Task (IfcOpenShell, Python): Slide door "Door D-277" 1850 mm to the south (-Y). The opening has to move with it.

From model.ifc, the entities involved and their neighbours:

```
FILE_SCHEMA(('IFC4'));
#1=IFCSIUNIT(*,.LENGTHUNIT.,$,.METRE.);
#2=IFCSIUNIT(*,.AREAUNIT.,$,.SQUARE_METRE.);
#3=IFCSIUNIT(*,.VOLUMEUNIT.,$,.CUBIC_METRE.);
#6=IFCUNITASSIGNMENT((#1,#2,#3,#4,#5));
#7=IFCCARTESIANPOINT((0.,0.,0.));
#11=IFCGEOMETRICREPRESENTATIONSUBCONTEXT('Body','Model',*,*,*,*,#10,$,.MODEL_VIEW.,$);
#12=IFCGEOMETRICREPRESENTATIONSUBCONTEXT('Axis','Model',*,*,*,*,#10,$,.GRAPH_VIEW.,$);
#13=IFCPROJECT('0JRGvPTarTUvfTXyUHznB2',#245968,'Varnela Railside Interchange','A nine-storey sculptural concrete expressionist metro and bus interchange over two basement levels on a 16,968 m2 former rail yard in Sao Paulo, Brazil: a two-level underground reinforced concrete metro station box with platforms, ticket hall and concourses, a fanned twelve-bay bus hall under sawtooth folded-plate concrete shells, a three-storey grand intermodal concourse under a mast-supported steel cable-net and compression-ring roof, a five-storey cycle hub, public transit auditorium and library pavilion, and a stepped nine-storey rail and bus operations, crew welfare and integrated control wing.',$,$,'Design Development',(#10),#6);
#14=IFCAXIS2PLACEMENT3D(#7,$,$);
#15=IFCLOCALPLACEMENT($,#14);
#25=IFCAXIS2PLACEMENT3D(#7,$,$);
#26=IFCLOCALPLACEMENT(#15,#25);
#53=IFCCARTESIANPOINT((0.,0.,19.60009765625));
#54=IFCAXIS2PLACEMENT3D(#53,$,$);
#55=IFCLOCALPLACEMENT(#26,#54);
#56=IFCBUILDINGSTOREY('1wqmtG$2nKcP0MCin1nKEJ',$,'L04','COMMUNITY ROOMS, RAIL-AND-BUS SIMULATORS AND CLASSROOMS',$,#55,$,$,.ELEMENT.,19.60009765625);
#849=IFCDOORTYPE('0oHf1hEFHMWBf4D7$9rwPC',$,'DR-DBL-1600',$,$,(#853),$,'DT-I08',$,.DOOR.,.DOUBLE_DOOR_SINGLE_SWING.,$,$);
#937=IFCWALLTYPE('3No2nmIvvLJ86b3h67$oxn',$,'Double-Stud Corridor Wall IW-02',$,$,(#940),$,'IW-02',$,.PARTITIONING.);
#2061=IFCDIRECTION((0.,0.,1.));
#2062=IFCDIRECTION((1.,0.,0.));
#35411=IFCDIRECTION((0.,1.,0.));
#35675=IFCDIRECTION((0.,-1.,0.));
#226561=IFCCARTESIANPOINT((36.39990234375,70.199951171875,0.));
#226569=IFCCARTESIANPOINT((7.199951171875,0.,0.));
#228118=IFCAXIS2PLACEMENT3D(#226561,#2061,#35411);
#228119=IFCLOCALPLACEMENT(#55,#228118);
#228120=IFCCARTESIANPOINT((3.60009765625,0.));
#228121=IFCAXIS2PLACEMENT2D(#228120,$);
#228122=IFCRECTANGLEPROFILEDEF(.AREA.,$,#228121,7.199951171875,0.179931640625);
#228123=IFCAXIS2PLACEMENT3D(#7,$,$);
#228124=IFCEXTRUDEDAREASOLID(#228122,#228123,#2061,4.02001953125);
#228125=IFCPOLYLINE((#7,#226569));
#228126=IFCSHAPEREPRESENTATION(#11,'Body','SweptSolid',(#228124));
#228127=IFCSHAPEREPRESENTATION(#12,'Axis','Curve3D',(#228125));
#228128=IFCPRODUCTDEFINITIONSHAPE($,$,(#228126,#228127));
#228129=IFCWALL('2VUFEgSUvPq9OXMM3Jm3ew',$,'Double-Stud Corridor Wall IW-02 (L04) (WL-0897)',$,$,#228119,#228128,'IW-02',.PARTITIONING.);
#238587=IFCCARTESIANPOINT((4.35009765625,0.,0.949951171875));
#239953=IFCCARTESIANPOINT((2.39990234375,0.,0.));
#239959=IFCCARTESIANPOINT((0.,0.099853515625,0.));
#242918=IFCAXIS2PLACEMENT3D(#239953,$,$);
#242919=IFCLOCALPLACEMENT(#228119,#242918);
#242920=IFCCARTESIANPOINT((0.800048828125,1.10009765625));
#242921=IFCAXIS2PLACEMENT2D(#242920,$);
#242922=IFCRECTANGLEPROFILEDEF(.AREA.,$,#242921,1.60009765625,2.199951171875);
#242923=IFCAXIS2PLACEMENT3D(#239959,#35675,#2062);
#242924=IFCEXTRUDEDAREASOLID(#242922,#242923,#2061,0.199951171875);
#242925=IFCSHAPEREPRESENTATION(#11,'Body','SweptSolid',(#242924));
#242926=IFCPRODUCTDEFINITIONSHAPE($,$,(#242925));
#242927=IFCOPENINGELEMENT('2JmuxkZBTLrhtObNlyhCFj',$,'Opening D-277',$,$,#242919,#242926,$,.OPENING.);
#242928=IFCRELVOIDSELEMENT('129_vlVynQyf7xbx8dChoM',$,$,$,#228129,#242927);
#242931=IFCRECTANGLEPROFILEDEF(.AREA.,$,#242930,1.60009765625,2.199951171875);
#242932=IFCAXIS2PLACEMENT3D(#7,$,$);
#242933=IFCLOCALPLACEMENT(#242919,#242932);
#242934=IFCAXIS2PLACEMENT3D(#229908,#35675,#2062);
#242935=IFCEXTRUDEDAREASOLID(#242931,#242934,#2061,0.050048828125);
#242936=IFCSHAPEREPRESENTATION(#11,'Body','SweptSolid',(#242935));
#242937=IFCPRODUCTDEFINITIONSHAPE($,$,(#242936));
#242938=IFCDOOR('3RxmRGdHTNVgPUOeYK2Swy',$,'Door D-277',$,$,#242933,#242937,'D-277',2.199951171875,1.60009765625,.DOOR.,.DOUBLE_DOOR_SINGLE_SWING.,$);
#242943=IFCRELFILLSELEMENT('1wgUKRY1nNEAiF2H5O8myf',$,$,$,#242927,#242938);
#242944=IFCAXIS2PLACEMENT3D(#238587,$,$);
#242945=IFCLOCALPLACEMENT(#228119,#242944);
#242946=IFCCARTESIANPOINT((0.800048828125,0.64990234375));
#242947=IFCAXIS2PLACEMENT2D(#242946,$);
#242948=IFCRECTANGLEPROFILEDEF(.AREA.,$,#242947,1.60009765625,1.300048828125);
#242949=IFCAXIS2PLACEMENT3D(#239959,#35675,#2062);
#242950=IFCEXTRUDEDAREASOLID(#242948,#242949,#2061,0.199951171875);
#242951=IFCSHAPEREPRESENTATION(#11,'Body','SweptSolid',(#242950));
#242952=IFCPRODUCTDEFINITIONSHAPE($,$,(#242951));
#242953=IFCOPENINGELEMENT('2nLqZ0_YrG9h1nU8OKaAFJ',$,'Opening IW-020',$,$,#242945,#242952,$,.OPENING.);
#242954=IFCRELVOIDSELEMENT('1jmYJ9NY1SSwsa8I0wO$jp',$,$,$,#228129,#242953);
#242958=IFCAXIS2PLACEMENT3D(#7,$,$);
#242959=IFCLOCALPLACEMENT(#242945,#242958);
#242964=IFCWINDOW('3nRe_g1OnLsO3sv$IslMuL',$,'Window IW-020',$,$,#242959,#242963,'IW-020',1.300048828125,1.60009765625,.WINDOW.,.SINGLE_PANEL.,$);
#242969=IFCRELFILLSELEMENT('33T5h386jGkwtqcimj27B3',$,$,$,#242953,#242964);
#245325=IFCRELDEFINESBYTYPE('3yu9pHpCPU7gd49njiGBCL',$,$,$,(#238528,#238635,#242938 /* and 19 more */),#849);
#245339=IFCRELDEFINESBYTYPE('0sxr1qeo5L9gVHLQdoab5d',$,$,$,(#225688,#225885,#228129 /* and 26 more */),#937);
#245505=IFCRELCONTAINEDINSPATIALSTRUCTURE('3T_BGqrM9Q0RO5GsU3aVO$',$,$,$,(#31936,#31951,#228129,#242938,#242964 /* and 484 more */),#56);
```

```python
import ifcopenshell
import ifcopenshell.api.geometry
import ifcopenshell.util.placement
import ifcopenshell.util.unit

model = ifcopenshell.open("model.ifc")
unit_scale = ifcopenshell.util.unit.calculate_unit_scale(model)

door = model.by_id(242938)
opening = door.FillsVoids[0].RelatingOpeningElement
wall = opening.VoidsElements[0].RelatingBuildingElement

wall_matrix = ifcopenshell.util.placement.get_local_placement(wall.ObjectPlacement)
shift = wall_matrix[:3, 0] * -1.85 / unit_scale
before = ifcopenshell.util.placement.get_local_placement(door.ObjectPlacement)[:3, 3].copy()

# The door is placed relative to its opening, so it follows when the opening moves.
matrix = ifcopenshell.util.placement.get_local_placement(opening.ObjectPlacement)
matrix[:3, 3] += shift
ifcopenshell.api.geometry.edit_object_placement(
    model, product=opening, matrix=matrix, is_si=False, should_transform_children=True
)

after = ifcopenshell.util.placement.get_local_placement(door.ObjectPlacement)[:3, 3]
print("door moved by", (after - before).round(3) + 0.0)

model.write("model_v2.ifc")
```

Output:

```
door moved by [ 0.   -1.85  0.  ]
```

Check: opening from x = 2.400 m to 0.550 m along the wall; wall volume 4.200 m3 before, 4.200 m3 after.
